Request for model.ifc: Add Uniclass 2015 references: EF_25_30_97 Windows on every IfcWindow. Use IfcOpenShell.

First a look at what the model holds.

```python
import ifcopenshell

model = ifcopenshell.open("model.ifc")
print(model.schema)
print("classifications:", [c.Name for c in model.by_type("IfcClassification")])
for ifc_class in ("IfcDoor", "IfcRoof", "IfcStair", "IfcWall", "IfcWindow"):
    print(ifc_class, len(model.by_type(ifc_class)))
```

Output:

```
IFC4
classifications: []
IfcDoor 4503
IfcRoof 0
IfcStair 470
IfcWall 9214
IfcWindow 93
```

```python
import ifcopenshell
import ifcopenshell.api.classification

model = ifcopenshell.open("model.ifc")

system = ifcopenshell.api.classification.add_classification(model, classification="Uniclass 2015")

codes = {
    "IfcWindow": ("EF_25_30_97", "Windows"),
}
for ifc_class, (code, name) in codes.items():
    products = model.by_type(ifc_class)
    ifcopenshell.api.classification.add_reference(
        model, products=products, classification=system, identification=code, name=name
    )
    print(code, len(products))

model.write("model_rev.ifc")
```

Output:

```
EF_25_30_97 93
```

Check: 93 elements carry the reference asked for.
